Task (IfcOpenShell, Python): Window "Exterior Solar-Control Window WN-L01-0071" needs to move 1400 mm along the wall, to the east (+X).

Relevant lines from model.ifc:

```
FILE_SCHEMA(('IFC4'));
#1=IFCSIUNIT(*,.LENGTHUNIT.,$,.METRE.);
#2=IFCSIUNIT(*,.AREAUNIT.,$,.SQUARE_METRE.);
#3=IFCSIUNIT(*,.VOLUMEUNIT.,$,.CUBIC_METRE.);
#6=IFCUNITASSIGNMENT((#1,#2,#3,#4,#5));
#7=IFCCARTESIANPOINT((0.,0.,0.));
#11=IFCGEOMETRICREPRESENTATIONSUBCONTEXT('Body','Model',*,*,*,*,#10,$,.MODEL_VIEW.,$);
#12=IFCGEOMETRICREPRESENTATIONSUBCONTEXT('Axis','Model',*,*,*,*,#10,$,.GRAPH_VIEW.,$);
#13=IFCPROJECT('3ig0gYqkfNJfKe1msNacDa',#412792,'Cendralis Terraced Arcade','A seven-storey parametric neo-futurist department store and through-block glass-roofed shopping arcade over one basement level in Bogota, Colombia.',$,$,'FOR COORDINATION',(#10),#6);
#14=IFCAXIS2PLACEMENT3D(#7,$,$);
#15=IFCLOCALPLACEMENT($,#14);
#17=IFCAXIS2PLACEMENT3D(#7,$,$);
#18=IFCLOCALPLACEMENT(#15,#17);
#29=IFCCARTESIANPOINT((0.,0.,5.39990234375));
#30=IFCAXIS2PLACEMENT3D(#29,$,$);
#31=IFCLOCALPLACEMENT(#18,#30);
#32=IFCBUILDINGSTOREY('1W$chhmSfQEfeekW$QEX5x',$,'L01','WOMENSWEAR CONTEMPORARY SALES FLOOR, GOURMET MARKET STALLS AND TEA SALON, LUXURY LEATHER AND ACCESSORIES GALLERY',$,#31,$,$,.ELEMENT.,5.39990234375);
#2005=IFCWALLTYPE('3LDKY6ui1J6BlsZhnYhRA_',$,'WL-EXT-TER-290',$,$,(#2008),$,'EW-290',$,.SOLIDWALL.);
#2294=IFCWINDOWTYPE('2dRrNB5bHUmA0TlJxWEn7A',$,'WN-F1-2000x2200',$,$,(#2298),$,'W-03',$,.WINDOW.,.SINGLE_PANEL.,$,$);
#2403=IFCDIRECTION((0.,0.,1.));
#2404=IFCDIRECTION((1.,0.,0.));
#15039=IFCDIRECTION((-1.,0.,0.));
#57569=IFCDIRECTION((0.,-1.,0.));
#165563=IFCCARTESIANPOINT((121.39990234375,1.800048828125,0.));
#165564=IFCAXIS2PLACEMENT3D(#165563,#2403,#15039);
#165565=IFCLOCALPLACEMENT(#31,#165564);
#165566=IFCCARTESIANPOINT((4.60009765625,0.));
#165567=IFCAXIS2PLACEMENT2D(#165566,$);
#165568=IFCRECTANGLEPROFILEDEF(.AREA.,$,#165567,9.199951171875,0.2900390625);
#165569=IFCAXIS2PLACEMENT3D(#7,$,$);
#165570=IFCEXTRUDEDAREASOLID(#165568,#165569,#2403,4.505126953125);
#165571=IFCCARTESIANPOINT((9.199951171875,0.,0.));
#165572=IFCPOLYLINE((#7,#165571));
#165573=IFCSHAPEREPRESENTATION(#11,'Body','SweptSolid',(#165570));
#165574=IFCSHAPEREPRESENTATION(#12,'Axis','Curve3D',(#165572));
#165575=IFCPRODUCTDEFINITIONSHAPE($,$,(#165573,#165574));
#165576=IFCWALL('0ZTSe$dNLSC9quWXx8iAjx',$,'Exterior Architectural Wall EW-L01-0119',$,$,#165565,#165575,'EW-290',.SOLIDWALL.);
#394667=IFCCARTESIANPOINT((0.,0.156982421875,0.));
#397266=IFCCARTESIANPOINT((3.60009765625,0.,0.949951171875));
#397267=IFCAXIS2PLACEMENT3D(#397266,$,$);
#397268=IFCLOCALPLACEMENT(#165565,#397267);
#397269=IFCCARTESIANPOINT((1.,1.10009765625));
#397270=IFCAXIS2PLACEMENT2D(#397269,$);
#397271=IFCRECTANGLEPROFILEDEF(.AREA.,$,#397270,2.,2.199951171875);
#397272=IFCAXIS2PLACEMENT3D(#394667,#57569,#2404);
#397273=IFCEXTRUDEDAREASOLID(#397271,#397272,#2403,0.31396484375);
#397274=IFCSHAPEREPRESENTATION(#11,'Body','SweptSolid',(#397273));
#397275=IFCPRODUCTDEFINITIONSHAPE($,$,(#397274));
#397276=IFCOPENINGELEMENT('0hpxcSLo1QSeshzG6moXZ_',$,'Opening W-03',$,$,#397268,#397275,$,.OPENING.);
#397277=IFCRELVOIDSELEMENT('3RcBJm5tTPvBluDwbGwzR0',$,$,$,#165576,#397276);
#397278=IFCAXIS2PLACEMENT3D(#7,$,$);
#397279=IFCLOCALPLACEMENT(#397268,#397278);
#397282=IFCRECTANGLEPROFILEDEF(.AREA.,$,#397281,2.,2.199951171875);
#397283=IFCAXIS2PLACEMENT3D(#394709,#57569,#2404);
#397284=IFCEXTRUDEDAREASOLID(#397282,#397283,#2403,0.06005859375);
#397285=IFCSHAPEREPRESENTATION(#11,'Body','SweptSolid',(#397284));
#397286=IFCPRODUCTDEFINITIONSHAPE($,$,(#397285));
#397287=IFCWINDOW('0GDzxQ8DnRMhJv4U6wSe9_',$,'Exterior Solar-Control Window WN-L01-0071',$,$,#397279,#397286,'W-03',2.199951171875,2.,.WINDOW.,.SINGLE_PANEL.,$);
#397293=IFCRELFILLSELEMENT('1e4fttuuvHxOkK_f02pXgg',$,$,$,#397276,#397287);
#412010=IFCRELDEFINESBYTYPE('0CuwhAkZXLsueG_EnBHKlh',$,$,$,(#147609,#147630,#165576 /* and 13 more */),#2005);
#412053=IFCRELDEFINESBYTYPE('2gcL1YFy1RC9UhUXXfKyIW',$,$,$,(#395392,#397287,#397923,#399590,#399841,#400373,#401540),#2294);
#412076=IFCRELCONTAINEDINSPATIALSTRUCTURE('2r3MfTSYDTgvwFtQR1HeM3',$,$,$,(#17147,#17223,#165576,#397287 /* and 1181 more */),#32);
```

```python
import ifcopenshell
import ifcopenshell.api.geometry
import ifcopenshell.util.placement
import ifcopenshell.util.unit

model = ifcopenshell.open("model.ifc")
unit_scale = ifcopenshell.util.unit.calculate_unit_scale(model)

window = model.by_guid("0GDzxQ8DnRMhJv4U6wSe9_")
opening = window.FillsVoids[0].RelatingOpeningElement
wall = opening.VoidsElements[0].RelatingBuildingElement

wall_matrix = ifcopenshell.util.placement.get_local_placement(wall.ObjectPlacement)
shift = wall_matrix[:3, 0] * -1.4 / unit_scale
before = ifcopenshell.util.placement.get_local_placement(window.ObjectPlacement)[:3, 3].copy()

# The window is placed relative to its opening, so it follows when the opening moves.
matrix = ifcopenshell.util.placement.get_local_placement(opening.ObjectPlacement)
matrix[:3, 3] += shift
ifcopenshell.api.geometry.edit_object_placement(
    model, product=opening, matrix=matrix, is_si=False, should_transform_children=True
)

after = ifcopenshell.util.placement.get_local_placement(window.ObjectPlacement)[:3, 3]
print("window moved by", (after - before).round(3) + 0.0)

model.write("model_edited.ifc")
```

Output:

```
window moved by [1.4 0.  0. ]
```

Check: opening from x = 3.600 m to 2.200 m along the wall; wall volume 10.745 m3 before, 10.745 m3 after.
